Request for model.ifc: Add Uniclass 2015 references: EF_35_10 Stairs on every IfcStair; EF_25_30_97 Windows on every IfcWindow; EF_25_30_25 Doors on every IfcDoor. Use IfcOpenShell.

First a look at what the model holds.

```python
import ifcopenshell

model = ifcopenshell.open("model.ifc")
print(model.schema)
print("classifications:", [c.Name for c in model.by_type("IfcClassification")])
for ifc_class in ("IfcDoor", "IfcRoof", "IfcStair", "IfcWall", "IfcWindow"):
    print(ifc_class, len(model.by_type(ifc_class)))
```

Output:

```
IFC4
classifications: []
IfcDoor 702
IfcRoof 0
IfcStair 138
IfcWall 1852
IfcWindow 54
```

```python
import ifcopenshell
import ifcopenshell.api.classification

model = ifcopenshell.open("model.ifc")

system = ifcopenshell.api.classification.add_classification(model, classification="Uniclass 2015")

codes = {
    "IfcStair": ("EF_35_10", "Stairs"),
    "IfcWindow": ("EF_25_30_97", "Windows"),
    "IfcDoor": ("EF_25_30_25", "Doors"),
}
for ifc_class, (code, name) in codes.items():
    products = model.by_type(ifc_class)
    ifcopenshell.api.classification.add_reference(
        model, products=products, classification=system, identification=code, name=name
    )
    print(code, len(products))

model.write("model_edited.ifc")
```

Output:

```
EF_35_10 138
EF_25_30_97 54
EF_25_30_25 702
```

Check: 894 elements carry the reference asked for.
